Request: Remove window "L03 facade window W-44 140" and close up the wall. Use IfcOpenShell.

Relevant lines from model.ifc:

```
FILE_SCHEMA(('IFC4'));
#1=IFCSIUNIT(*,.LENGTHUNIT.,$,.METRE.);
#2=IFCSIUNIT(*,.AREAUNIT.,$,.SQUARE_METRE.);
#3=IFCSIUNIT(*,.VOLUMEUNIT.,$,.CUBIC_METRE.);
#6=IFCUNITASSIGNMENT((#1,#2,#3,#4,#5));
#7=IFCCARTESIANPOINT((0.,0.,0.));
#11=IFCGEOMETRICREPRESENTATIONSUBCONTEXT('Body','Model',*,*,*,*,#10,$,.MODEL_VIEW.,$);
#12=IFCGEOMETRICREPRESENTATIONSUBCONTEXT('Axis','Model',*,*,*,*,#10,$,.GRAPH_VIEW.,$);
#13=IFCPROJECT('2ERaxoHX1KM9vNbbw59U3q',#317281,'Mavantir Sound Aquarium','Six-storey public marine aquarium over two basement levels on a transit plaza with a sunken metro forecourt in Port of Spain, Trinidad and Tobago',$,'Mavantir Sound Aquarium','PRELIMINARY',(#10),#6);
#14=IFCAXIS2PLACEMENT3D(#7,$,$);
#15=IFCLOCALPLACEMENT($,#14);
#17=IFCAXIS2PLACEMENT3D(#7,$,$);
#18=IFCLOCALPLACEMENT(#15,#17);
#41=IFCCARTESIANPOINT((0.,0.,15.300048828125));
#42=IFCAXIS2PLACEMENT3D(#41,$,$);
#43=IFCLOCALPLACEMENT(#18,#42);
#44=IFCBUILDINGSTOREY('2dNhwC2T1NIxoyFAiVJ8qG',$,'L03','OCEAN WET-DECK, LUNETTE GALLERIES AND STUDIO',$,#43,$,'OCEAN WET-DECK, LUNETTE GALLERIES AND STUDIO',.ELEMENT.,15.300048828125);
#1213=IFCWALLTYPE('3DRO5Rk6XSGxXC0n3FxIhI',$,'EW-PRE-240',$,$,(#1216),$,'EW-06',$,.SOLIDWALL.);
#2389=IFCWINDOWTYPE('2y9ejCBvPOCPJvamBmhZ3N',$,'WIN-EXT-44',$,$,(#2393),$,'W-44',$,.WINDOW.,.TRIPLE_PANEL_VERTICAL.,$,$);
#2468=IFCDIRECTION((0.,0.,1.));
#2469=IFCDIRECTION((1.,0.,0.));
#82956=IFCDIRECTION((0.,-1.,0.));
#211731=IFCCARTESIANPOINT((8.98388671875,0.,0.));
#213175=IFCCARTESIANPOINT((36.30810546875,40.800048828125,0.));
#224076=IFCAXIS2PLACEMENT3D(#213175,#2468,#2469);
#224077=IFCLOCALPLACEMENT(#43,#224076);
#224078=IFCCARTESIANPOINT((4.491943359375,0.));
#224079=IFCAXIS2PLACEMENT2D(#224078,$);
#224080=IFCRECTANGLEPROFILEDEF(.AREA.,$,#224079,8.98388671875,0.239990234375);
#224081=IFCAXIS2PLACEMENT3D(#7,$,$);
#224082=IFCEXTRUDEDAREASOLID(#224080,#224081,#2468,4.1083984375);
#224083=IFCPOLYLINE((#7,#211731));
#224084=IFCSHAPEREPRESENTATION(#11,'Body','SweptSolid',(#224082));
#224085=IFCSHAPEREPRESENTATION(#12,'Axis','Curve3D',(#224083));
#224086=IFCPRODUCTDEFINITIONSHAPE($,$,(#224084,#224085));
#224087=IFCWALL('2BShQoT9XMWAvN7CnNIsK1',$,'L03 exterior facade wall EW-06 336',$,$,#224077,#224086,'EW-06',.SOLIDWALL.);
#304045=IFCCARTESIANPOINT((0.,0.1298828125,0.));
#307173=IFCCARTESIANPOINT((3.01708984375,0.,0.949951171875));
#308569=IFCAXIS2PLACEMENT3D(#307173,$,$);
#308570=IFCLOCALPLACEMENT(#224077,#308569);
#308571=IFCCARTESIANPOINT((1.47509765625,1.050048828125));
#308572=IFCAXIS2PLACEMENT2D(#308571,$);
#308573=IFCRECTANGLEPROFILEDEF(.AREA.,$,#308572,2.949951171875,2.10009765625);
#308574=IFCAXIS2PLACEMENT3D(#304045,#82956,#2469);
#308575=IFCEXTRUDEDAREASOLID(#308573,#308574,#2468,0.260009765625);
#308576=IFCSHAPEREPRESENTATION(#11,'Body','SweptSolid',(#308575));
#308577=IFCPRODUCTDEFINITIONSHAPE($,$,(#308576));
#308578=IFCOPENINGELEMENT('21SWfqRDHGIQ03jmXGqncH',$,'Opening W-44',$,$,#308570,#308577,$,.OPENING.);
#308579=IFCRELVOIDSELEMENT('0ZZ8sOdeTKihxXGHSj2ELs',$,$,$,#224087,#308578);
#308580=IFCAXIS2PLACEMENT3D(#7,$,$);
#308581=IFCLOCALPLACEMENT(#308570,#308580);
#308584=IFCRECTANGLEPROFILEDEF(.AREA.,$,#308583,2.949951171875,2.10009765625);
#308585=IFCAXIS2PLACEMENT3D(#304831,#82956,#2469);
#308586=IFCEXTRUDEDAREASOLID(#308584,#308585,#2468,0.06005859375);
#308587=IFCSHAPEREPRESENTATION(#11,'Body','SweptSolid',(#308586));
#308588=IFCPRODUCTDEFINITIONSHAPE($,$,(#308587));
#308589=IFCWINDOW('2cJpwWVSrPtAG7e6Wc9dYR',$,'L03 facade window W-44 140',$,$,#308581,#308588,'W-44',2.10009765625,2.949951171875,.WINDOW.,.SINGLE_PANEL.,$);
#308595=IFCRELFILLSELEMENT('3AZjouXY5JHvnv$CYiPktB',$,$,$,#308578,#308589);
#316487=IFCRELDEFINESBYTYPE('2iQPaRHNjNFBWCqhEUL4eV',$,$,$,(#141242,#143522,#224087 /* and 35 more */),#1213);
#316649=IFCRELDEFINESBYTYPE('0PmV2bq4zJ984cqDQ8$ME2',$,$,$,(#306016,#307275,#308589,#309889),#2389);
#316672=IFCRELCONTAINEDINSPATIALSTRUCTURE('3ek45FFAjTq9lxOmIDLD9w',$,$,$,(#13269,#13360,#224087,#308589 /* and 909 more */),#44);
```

```python
import ifcopenshell
import ifcopenshell.api.feature
import ifcopenshell.api.root
import ifcopenshell.geom
import ifcopenshell.util.shape

model = ifcopenshell.open("model.ifc")
settings = ifcopenshell.geom.settings()


def volume(element):
    """Net volume in cubic metres, openings subtracted."""
    shape = ifcopenshell.geom.create_shape(settings, element)
    return ifcopenshell.util.shape.get_volume(shape.geometry)


window = model.by_id(308589)
opening = window.FillsVoids[0].RelatingOpeningElement
wall = opening.VoidsElements[0].RelatingBuildingElement
before = volume(wall)

ifcopenshell.api.root.remove_product(model, product=window)
ifcopenshell.api.feature.remove_feature(model, feature=opening)

after = volume(wall)

print(f"wall volume {before:.3f} -> {after:.3f} m3")

model.write("model-out.ifc")
```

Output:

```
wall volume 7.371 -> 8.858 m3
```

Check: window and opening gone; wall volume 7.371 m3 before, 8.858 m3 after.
